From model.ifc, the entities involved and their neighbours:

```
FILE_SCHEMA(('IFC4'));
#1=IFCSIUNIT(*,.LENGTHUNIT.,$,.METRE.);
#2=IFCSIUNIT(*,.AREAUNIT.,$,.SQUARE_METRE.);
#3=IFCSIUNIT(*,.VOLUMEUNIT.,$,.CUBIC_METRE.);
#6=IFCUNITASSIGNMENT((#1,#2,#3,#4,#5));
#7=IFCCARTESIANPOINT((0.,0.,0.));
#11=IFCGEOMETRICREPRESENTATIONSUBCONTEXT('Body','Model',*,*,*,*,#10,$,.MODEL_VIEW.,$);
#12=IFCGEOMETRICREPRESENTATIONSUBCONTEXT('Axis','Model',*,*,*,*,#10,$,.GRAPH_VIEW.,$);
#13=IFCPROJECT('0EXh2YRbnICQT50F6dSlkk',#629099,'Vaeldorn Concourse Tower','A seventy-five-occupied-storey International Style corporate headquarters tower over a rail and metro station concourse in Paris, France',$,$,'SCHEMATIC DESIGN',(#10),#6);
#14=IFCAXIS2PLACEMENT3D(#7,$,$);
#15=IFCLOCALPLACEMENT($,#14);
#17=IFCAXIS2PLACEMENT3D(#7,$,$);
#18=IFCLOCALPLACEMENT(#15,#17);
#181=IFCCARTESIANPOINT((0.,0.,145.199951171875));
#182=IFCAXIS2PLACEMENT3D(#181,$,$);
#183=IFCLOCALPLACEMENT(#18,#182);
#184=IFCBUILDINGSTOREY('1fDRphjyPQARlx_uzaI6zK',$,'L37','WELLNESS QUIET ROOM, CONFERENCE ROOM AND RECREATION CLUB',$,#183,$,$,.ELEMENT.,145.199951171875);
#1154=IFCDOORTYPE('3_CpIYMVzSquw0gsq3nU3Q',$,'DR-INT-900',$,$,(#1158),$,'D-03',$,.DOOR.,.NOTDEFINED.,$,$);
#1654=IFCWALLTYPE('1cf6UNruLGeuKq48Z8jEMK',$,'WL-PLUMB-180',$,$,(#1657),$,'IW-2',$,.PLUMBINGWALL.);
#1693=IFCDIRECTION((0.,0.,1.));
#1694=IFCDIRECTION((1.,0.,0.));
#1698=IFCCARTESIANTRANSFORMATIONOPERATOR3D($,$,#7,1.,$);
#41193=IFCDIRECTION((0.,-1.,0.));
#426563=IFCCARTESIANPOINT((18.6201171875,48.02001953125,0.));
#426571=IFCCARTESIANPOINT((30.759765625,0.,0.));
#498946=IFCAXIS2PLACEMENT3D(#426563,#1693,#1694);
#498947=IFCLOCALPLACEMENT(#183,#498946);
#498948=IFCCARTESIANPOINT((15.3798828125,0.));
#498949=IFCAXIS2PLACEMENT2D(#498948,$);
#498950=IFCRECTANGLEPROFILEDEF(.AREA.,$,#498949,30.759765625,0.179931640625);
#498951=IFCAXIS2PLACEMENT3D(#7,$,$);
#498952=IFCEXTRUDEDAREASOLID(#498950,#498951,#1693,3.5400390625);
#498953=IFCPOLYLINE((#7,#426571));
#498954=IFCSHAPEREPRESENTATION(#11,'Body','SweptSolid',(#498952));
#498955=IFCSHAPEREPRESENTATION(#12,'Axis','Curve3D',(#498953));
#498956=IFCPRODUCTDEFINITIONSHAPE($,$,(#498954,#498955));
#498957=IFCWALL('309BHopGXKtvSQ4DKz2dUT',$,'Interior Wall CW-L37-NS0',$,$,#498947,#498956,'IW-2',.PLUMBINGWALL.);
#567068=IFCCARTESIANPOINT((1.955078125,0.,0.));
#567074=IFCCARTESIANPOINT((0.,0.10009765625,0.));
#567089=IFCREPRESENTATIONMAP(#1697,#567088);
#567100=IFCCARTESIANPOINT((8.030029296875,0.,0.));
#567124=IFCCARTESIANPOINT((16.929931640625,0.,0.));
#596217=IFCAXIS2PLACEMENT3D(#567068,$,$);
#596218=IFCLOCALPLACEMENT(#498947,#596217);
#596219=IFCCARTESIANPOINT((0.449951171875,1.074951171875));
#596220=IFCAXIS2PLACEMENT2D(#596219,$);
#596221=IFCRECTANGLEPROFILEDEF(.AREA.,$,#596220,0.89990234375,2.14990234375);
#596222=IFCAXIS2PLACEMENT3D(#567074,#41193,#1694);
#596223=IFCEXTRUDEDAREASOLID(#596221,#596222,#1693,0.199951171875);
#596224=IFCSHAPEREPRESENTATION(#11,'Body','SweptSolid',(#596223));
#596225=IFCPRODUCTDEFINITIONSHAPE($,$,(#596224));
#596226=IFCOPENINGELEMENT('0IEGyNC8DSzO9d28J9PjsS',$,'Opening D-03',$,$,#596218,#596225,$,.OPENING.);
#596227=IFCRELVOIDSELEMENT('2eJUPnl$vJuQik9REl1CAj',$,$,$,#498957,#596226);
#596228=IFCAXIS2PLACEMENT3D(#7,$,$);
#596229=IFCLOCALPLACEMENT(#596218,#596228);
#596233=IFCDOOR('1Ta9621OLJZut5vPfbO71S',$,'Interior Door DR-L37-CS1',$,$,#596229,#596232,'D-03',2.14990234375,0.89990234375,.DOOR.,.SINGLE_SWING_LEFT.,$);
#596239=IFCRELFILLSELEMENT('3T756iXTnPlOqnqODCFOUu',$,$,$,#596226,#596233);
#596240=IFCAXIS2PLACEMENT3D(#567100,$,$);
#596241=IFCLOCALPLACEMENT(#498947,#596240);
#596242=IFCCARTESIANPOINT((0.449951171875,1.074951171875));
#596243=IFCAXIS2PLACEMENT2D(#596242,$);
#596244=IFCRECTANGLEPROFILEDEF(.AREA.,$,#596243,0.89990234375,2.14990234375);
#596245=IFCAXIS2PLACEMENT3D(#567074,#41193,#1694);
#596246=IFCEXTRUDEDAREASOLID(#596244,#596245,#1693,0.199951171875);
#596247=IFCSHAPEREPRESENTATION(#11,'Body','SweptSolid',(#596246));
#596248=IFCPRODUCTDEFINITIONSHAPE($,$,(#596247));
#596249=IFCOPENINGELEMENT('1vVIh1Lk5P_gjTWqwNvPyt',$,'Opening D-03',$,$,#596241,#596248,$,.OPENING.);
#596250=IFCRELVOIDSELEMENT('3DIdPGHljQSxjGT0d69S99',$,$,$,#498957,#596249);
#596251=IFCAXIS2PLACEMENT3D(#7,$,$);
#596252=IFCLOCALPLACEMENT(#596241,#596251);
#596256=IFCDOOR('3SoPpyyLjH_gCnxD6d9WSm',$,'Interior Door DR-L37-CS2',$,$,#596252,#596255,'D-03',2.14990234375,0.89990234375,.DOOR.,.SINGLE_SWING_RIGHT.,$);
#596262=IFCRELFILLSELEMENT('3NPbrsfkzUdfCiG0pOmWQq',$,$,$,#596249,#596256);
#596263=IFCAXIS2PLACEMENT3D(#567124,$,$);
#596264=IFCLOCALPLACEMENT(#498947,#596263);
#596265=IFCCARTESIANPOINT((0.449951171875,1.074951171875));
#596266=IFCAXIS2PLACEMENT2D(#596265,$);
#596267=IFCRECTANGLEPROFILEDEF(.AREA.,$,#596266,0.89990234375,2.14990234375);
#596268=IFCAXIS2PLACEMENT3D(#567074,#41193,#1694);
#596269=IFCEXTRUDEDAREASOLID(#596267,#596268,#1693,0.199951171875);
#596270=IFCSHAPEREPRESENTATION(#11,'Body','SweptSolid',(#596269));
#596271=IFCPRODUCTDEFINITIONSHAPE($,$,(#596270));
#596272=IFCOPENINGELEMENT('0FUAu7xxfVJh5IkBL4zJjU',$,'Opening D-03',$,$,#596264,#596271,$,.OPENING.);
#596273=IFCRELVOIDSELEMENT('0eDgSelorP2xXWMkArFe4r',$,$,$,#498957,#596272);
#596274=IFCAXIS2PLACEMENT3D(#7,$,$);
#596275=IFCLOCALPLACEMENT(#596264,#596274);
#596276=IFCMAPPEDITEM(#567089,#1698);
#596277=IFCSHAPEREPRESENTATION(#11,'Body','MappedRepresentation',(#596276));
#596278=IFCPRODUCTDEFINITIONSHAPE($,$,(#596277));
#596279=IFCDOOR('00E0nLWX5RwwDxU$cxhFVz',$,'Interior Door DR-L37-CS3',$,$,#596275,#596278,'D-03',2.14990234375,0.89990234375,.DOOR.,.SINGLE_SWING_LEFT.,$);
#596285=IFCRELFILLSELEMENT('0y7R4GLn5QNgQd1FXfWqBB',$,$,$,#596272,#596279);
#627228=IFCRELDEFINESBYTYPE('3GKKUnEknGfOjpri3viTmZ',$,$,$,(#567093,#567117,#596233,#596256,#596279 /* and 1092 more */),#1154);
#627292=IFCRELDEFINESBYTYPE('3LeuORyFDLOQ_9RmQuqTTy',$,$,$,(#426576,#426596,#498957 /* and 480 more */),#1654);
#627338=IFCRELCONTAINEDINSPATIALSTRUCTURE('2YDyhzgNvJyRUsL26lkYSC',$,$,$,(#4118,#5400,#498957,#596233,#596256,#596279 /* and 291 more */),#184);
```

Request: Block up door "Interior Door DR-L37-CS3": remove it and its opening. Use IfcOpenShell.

```python
import ifcopenshell
import ifcopenshell.api.feature
import ifcopenshell.api.root
import ifcopenshell.geom
import ifcopenshell.util.shape

model = ifcopenshell.open("model.ifc")
settings = ifcopenshell.geom.settings()


def volume(element):
    """Net volume in cubic metres, openings subtracted."""
    shape = ifcopenshell.geom.create_shape(settings, element)
    return ifcopenshell.util.shape.get_volume(shape.geometry)


door = model.by_guid("00E0nLWX5RwwDxU$cxhFVz")
opening = door.FillsVoids[0].RelatingOpeningElement
wall = opening.VoidsElements[0].RelatingBuildingElement
before = volume(wall)

ifcopenshell.api.root.remove_product(model, product=door)
ifcopenshell.api.feature.remove_feature(model, feature=opening)

after = volume(wall)

print(f"wall volume {before:.3f} -> {after:.3f} m3")

model.write("model_updated.ifc")
```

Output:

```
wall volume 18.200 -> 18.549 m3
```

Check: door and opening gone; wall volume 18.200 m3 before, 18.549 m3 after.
